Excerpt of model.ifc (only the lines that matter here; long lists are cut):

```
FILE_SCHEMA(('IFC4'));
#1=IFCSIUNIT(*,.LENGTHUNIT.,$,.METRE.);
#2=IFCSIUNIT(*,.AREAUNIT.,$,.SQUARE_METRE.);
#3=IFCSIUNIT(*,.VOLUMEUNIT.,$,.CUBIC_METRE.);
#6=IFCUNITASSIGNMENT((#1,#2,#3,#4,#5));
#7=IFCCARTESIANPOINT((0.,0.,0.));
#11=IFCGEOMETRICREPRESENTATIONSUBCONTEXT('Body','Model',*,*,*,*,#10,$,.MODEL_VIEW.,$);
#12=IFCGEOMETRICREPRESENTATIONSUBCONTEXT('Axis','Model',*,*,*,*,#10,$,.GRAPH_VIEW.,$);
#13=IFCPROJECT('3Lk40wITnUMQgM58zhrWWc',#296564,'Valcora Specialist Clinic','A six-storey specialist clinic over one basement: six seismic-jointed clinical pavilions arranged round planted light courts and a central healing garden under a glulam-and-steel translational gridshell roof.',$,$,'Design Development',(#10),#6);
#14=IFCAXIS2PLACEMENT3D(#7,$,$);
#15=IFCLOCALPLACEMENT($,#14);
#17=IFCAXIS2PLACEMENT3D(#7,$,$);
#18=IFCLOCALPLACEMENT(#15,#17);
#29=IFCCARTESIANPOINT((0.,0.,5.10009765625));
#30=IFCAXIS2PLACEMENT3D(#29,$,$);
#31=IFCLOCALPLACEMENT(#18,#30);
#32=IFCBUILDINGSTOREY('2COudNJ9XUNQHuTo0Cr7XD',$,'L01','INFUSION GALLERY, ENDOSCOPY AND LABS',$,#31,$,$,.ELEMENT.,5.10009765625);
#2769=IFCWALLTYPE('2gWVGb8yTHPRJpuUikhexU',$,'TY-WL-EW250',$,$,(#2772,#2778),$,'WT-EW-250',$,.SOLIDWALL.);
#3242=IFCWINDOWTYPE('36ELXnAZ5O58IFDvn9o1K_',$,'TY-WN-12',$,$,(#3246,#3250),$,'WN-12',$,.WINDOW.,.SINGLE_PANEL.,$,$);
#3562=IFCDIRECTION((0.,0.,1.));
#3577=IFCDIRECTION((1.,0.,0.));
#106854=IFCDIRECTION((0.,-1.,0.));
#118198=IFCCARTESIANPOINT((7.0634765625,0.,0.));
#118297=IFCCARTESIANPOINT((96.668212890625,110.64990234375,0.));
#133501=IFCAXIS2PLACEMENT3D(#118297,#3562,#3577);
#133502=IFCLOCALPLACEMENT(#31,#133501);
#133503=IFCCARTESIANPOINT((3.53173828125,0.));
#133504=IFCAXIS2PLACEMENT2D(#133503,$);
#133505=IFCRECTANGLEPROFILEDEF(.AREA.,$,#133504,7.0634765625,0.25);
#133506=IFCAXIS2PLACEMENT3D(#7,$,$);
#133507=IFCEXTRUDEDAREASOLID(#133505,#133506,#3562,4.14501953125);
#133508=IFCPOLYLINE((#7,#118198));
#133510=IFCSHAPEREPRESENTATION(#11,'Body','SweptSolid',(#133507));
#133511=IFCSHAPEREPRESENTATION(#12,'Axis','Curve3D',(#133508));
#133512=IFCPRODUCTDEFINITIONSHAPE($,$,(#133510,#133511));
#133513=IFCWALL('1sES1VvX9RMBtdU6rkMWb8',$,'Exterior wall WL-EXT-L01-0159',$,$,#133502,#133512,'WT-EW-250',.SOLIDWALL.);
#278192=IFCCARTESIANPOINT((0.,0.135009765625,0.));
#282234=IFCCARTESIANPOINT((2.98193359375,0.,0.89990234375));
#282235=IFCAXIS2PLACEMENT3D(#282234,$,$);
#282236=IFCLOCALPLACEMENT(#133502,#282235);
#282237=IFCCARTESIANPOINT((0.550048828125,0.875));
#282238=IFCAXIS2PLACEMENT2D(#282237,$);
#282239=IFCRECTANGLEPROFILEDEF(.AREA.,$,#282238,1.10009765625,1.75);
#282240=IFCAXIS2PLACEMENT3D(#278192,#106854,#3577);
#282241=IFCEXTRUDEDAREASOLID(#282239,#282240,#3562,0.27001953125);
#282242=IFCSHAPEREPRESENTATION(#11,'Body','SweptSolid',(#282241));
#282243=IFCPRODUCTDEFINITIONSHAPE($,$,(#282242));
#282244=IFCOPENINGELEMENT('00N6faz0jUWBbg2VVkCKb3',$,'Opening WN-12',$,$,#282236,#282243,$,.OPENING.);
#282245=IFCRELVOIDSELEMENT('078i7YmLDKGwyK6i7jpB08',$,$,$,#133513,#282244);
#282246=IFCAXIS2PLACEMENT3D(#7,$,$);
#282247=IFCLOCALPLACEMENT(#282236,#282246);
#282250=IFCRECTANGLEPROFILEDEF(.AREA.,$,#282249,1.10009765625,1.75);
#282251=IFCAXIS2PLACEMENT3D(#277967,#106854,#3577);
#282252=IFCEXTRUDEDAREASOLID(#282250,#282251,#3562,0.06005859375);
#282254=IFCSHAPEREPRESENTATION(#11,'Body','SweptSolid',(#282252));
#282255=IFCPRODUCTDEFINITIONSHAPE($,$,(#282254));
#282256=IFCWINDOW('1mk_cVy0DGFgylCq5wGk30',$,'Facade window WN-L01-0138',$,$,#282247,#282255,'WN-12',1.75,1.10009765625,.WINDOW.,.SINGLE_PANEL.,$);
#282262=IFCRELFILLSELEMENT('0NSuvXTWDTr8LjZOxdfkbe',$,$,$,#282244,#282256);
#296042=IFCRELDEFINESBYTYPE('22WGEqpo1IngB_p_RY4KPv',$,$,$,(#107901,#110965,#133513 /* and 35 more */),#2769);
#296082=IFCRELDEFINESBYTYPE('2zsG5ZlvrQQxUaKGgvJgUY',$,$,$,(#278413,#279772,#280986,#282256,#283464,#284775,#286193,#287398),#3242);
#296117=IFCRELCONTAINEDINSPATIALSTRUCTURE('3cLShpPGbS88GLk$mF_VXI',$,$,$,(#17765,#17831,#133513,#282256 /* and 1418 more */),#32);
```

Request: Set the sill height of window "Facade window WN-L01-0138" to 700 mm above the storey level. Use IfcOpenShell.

```python
import numpy as np
import ifcopenshell
import ifcopenshell.api.geometry
import ifcopenshell.geom
import ifcopenshell.util.element
import ifcopenshell.util.placement
import ifcopenshell.util.shape
import ifcopenshell.util.unit

model = ifcopenshell.open("model.ifc")
unit_scale = ifcopenshell.util.unit.calculate_unit_scale(model)

window = model.by_id(282256)
opening = window.FillsVoids[0].RelatingOpeningElement
storey = ifcopenshell.util.element.get_container(window, ifc_class="IfcBuildingStorey")
level = ifcopenshell.util.placement.get_local_placement(storey.ObjectPlacement)[2, 3]

# The opening's origin need not be at the sill, so measure its lowest point.
shape = ifcopenshell.geom.create_shape(ifcopenshell.geom.settings(), opening)
bottom = ifcopenshell.util.shape.get_shape_bottom_elevation(shape, shape.geometry) / unit_scale
dz = level + 0.7 - bottom

shift = np.array([0.0, 0.0, dz])
# The window is placed relative to its opening, so it follows when the opening moves.
matrix = ifcopenshell.util.placement.get_local_placement(opening.ObjectPlacement)
matrix[:3, 3] += shift
ifcopenshell.api.geometry.edit_object_placement(
    model, product=opening, matrix=matrix, is_si=False, should_transform_children=True
)

print(f"moved by {dz * unit_scale:+.3f} m")

model.write("model_v2.ifc")
```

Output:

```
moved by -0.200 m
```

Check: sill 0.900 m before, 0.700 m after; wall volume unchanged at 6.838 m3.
